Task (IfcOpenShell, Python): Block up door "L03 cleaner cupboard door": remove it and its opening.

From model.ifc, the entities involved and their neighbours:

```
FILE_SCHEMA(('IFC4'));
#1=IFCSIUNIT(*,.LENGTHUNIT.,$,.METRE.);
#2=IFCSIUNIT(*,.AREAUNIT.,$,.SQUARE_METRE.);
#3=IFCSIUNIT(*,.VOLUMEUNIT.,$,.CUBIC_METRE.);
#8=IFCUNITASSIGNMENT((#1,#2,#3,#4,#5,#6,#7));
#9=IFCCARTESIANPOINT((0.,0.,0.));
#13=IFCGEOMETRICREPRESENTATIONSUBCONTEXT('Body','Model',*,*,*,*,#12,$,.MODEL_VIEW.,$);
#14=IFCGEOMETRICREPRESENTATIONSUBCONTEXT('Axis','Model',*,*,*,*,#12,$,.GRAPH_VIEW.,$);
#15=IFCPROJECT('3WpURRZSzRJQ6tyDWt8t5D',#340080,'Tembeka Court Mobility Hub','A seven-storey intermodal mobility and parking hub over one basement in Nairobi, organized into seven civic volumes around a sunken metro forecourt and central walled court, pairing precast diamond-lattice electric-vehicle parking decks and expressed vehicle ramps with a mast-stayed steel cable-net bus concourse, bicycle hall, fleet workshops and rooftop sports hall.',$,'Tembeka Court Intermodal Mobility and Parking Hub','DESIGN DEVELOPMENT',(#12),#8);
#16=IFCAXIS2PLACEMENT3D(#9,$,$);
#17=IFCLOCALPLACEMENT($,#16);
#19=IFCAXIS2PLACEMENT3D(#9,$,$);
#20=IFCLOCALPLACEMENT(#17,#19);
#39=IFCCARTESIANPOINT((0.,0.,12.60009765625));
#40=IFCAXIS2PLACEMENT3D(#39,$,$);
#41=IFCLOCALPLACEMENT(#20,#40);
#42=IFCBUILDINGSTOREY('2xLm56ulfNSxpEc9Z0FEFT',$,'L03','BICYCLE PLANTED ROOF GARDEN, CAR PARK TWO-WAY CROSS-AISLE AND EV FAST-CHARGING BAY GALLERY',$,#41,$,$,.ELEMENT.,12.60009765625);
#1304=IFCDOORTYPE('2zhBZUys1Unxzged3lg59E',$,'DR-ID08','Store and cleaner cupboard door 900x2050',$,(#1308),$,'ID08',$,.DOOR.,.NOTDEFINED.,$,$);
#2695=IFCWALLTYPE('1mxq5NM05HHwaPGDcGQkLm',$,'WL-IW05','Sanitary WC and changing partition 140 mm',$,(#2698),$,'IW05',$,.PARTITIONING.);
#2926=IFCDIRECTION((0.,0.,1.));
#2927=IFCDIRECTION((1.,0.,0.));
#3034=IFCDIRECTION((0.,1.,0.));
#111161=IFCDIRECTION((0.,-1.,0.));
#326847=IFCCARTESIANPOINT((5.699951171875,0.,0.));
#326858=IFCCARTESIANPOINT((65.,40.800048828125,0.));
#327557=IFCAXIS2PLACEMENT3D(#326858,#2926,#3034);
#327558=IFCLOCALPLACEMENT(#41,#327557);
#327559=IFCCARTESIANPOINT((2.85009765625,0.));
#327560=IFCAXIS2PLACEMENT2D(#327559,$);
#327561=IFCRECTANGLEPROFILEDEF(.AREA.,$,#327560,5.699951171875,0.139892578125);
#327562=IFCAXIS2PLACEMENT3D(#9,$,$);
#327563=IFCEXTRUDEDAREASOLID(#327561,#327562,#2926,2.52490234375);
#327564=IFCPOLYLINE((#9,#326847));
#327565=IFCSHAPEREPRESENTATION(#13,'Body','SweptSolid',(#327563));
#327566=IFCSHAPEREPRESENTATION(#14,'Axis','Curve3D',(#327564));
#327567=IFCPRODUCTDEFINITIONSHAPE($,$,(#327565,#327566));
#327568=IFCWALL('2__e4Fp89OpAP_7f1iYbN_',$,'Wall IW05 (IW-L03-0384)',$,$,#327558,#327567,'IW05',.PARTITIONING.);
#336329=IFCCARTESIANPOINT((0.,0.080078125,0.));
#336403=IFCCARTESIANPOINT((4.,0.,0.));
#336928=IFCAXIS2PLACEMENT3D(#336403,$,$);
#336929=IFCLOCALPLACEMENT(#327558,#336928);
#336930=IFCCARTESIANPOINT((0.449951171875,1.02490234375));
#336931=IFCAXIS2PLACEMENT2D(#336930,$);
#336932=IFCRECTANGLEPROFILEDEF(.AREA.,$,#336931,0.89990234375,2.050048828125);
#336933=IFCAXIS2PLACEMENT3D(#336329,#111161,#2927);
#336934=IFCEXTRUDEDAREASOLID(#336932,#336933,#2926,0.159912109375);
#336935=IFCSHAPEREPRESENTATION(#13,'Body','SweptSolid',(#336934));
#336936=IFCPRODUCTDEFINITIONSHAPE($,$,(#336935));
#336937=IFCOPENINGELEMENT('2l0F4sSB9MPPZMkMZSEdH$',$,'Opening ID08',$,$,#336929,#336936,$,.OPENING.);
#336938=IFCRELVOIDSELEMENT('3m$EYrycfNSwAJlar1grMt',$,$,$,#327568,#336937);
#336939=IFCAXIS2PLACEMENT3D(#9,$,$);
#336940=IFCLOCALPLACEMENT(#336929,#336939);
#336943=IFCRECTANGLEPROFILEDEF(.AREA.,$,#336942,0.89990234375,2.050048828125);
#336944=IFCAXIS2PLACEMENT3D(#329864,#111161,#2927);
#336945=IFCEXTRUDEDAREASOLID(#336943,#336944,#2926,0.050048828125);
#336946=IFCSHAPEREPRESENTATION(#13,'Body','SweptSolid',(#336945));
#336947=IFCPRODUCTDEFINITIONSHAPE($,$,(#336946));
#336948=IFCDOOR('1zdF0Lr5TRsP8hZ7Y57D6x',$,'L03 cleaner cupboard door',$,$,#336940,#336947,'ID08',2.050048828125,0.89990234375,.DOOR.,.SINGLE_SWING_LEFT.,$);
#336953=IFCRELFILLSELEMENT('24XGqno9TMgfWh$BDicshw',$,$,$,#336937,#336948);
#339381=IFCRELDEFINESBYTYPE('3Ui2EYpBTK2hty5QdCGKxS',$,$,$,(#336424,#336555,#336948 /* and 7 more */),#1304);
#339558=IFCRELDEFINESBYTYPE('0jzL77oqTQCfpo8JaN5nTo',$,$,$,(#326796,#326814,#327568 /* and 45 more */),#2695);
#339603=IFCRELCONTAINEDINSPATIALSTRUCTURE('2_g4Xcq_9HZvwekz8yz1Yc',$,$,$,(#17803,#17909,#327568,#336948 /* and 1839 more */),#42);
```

```python
import ifcopenshell
import ifcopenshell.api.feature
import ifcopenshell.api.root
import ifcopenshell.geom
import ifcopenshell.util.shape

model = ifcopenshell.open("model.ifc")
settings = ifcopenshell.geom.settings()


def volume(element):
    """Net volume in cubic metres, openings subtracted."""
    shape = ifcopenshell.geom.create_shape(settings, element)
    return ifcopenshell.util.shape.get_volume(shape.geometry)


door = model.by_guid("1zdF0Lr5TRsP8hZ7Y57D6x")
opening = door.FillsVoids[0].RelatingOpeningElement
wall = opening.VoidsElements[0].RelatingBuildingElement
before = volume(wall)

ifcopenshell.api.root.remove_product(model, product=door)
ifcopenshell.api.feature.remove_feature(model, feature=opening)

after = volume(wall)

print(f"wall volume {before:.3f} -> {after:.3f} m3")

model.write("model_rev.ifc")
```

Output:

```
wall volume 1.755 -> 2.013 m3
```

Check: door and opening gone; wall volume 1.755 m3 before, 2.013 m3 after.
